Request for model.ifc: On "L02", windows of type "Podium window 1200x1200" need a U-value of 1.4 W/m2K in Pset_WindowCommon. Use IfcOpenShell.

First a look at what the model holds.

```python
import ifcopenshell
import ifcopenshell.util.element

model = ifcopenshell.open("model.ifc")
print(model.schema)
storey = next(s for s in model.by_type("IfcBuildingStorey") if s.Name == "L02")
windows = [e for e in ifcopenshell.util.element.get_decomposition(storey) if e.is_a("IfcWindow")]
seen = {}
for e in windows:
    element_type = ifcopenshell.util.element.get_type(e)
    key = (element_type.Name if element_type != e and element_type else None, ifcopenshell.util.element.get_pset(e, "Pset_WindowCommon", "ThermalTransmittance"))
    seen[key] = seen.get(key, 0) + 1
for (name, value), count in sorted(seen.items(), key=str):
    print(count, "x", name, "|", value)
```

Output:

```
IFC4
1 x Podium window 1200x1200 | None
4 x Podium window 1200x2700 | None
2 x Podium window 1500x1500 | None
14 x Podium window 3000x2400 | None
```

```python
import ifcopenshell
import ifcopenshell.api.pset
import ifcopenshell.util.element

model = ifcopenshell.open("model.ifc")

storey = next(s for s in model.by_type("IfcBuildingStorey") if s.Name == "L02")
windows = [e for e in ifcopenshell.util.element.get_decomposition(storey) if e.is_a("IfcWindow")]

count = 0
for e in windows:
    element_type = ifcopenshell.util.element.get_type(e)
    if element_type in (None, e) or element_type.Name != "Podium window 1200x1200":
        continue
    # add_pset returns the element's existing set when there is one.
    pset = ifcopenshell.api.pset.add_pset(model, product=e, name="Pset_WindowCommon")
    ifcopenshell.api.pset.edit_pset(model, pset=pset, properties={"ThermalTransmittance": 1.4})
    count += 1

print(count, "windows updated")

model.write("model_rev.ifc")
```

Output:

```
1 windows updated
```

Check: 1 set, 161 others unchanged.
